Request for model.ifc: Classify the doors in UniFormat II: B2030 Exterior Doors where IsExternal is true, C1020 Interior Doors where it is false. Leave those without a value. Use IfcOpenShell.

First a look at what the model holds.

```python
import ifcopenshell
import ifcopenshell.util.element

model = ifcopenshell.open("model.ifc")
print(model.schema)
print("classifications:", [c.Name for c in model.by_type("IfcClassification")])
values = [ifcopenshell.util.element.get_pset(e, "Pset_DoorCommon", "IsExternal") for e in model.by_type("IfcDoor")]
for value in (True, False, None):
    print("IsExternal", value, values.count(value))
```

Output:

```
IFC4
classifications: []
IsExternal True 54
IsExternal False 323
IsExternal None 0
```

```python
import ifcopenshell
import ifcopenshell.api.classification
import ifcopenshell.util.element

model = ifcopenshell.open("model.ifc")

system = ifcopenshell.api.classification.add_classification(model, classification="UniFormat II")

doors = model.by_type("IfcDoor")
external = {e: ifcopenshell.util.element.get_pset(e, "Pset_DoorCommon", "IsExternal") for e in doors}
for flag, code, name in ((True, "B2030", "Exterior Doors"), (False, "C1020", "Interior Doors")):
    products = [e for e in doors if external[e] is flag]
    ifcopenshell.api.classification.add_reference(
        model, products=products, classification=system, identification=code, name=name
    )
    print(code, len(products))

model.write("model_edited.ifc")
```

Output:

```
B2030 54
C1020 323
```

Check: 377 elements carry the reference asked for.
